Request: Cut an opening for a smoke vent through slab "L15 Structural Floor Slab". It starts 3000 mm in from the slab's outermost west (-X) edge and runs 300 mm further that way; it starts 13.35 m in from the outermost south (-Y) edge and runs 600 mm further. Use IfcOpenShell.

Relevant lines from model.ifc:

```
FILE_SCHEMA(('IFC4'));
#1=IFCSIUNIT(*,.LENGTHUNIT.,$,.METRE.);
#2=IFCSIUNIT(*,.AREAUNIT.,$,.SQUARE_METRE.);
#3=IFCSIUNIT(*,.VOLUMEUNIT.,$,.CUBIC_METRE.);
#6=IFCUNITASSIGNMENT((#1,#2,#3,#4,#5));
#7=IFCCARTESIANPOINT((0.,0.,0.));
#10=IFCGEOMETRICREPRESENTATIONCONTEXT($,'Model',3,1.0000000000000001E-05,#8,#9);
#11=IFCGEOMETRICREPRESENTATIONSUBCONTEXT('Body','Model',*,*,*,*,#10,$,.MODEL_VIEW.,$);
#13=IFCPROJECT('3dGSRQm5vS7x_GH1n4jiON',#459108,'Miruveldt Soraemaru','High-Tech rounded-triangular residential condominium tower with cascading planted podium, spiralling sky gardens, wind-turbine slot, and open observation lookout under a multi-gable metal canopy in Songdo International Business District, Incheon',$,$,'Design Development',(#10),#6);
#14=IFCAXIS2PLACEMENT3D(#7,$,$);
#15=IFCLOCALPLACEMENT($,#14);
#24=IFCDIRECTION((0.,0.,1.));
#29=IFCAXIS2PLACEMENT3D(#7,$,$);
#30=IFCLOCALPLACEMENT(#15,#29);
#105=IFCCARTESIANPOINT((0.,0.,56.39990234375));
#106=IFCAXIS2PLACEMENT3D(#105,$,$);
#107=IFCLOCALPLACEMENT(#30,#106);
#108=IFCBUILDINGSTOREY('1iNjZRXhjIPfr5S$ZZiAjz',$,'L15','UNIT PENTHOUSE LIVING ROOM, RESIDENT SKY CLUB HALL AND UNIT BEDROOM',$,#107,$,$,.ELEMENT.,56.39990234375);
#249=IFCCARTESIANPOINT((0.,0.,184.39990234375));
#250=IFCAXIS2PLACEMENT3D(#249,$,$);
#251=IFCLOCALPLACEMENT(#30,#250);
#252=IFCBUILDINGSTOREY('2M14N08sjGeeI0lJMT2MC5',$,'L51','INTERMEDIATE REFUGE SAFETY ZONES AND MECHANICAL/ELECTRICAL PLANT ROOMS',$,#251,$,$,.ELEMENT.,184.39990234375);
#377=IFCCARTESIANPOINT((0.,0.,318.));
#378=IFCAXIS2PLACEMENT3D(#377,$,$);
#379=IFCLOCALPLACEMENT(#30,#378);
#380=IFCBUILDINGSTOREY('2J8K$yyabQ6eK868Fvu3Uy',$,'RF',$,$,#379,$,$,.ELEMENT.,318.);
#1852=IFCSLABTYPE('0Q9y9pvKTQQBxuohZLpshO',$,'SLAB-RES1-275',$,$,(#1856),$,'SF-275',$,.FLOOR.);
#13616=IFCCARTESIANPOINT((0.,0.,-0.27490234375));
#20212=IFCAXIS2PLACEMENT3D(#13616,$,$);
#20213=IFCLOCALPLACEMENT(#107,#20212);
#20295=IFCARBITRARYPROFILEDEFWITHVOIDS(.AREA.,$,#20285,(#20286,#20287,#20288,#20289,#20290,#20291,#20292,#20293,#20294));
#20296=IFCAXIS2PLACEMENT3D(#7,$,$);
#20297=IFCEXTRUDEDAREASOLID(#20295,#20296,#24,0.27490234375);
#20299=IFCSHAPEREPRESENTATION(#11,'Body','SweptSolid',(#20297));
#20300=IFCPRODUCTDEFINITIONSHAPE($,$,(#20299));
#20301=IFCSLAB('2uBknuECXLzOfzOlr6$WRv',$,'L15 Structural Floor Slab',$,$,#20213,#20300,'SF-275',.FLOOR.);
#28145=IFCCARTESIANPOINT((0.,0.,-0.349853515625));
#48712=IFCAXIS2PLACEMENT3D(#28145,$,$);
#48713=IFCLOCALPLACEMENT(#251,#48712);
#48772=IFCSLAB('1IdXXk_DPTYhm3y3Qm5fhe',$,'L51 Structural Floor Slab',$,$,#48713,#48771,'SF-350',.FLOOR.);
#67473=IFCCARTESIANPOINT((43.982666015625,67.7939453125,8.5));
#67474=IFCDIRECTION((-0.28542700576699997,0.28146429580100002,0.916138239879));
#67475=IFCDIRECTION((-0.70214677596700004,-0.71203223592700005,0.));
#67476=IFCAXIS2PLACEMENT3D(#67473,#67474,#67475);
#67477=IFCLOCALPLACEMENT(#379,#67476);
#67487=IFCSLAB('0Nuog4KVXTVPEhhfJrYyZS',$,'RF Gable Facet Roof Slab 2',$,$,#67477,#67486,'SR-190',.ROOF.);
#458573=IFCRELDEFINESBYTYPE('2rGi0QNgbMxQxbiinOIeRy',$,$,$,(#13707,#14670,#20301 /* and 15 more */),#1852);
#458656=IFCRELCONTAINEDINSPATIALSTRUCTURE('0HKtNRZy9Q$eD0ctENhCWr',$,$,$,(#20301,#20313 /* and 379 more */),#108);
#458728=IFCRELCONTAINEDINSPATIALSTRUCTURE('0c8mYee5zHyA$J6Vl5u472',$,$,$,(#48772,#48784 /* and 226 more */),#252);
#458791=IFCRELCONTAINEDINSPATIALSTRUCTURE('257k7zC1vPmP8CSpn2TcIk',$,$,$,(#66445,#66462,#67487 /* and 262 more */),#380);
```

```python
import numpy as np
import ifcopenshell
import ifcopenshell.api.feature
import ifcopenshell.api.geometry
import ifcopenshell.api.root
import ifcopenshell.geom
import ifcopenshell.util.placement
import ifcopenshell.util.representation
import ifcopenshell.util.shape
import ifcopenshell.util.unit

model = ifcopenshell.open("model.ifc")
unit_scale = ifcopenshell.util.unit.calculate_unit_scale(model)
settings = ifcopenshell.geom.settings()


def volume(element):
    """Net volume in cubic metres, openings subtracted."""
    shape = ifcopenshell.geom.create_shape(settings, element)
    return ifcopenshell.util.shape.get_volume(shape.geometry)


slab = model.by_guid("2uBknuECXLzOfzOlr6$WRv")
before = volume(slab)

# Extent in the slab's own axes, in metres. The edges named are its -X and -Y sides.
slab_shape = ifcopenshell.geom.create_shape(settings, slab)
vertices = ifcopenshell.util.shape.get_vertices(slab_shape.geometry)
x_min, y_min, bottom = vertices.min(axis=0)
top = vertices[:, 2].max()

opening = ifcopenshell.api.root.create_entity(model, ifc_class="IfcOpeningElement", name="Smoke vent opening", predefined_type="OPENING")
context = ifcopenshell.util.representation.get_context(model, "Model", "Body", "MODEL_VIEW")
width, depth = 0.3, 0.6
outline = [(0.0, 0.0), (width, 0.0), (width, depth), (0.0, depth), (0.0, 0.0)]
# Overshoot both faces by 50 mm so the cut is clean.
shape = ifcopenshell.api.geometry.add_slab_representation(
    model, context=context, depth=top - bottom + 0.1, polyline=outline
)
ifcopenshell.api.geometry.assign_representation(model, product=opening, representation=shape)

matrix = ifcopenshell.util.placement.get_local_placement(slab.ObjectPlacement)
matrix[:, 3] = matrix @ np.append(np.array([x_min + 3, y_min + 13.35, bottom - 0.05]) / unit_scale, 1.0)
ifcopenshell.api.geometry.edit_object_placement(model, product=opening, matrix=matrix, is_si=False)
ifcopenshell.api.feature.add_feature(model, feature=opening, element=slab)

after = volume(slab)

print(f"slab volume {before:.3f} -> {after:.3f} m3")

model.write("model_updated.ifc")
```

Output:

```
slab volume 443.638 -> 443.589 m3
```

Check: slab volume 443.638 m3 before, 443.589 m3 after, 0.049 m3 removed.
